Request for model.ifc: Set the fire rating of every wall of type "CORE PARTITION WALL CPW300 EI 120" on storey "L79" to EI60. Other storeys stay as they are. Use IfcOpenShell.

First a look at what the model holds.

```python
import ifcopenshell
import ifcopenshell.util.element

model = ifcopenshell.open("model.ifc")
print(model.schema)
storey = next(s for s in model.by_type("IfcBuildingStorey") if s.Name == "L79")
walls = [e for e in ifcopenshell.util.element.get_decomposition(storey) if e.is_a("IfcWall")]
seen = {}
for e in walls:
    element_type = ifcopenshell.util.element.get_type(e)
    key = (element_type.Name if element_type != e and element_type else None, ifcopenshell.util.element.get_pset(e, "Pset_WallCommon", "FireRating"))
    seen[key] = seen.get(key, 0) + 1
for (name, value), count in sorted(seen.items(), key=str):
    print(count, "x", name, "|", value)
```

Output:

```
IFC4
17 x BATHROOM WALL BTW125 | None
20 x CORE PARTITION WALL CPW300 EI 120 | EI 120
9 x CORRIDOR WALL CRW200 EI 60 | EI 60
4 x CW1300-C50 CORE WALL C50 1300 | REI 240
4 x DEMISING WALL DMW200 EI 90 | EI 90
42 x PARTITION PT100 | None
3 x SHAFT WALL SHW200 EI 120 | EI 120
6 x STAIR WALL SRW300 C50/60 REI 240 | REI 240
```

```python
import ifcopenshell
import ifcopenshell.api.pset
import ifcopenshell.util.element

model = ifcopenshell.open("model.ifc")

storey = next(s for s in model.by_type("IfcBuildingStorey") if s.Name == "L79")
walls = [e for e in ifcopenshell.util.element.get_decomposition(storey) if e.is_a("IfcWall")]

count = 0
for e in walls:
    element_type = ifcopenshell.util.element.get_type(e)
    if element_type in (None, e) or element_type.Name != "CORE PARTITION WALL CPW300 EI 120":
        continue
    found = ifcopenshell.util.element.get_pset(e, "Pset_WallCommon", should_inherit=False)
    if found:
        pset = model.by_id(found["id"])
        if len(ifcopenshell.util.element.get_elements_by_pset(pset)) > 1:
            pset = ifcopenshell.api.pset.unshare_pset(model, products=[e], pset=pset)[0]
    else:
        pset = ifcopenshell.api.pset.add_pset(model, product=e, name="Pset_WallCommon")
    ifcopenshell.api.pset.edit_pset(model, pset=pset, properties={"FireRating": "EI60"})
    count += 1

print(count, "walls updated")

model.write("model_updated.ifc")
```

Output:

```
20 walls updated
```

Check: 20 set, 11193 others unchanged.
